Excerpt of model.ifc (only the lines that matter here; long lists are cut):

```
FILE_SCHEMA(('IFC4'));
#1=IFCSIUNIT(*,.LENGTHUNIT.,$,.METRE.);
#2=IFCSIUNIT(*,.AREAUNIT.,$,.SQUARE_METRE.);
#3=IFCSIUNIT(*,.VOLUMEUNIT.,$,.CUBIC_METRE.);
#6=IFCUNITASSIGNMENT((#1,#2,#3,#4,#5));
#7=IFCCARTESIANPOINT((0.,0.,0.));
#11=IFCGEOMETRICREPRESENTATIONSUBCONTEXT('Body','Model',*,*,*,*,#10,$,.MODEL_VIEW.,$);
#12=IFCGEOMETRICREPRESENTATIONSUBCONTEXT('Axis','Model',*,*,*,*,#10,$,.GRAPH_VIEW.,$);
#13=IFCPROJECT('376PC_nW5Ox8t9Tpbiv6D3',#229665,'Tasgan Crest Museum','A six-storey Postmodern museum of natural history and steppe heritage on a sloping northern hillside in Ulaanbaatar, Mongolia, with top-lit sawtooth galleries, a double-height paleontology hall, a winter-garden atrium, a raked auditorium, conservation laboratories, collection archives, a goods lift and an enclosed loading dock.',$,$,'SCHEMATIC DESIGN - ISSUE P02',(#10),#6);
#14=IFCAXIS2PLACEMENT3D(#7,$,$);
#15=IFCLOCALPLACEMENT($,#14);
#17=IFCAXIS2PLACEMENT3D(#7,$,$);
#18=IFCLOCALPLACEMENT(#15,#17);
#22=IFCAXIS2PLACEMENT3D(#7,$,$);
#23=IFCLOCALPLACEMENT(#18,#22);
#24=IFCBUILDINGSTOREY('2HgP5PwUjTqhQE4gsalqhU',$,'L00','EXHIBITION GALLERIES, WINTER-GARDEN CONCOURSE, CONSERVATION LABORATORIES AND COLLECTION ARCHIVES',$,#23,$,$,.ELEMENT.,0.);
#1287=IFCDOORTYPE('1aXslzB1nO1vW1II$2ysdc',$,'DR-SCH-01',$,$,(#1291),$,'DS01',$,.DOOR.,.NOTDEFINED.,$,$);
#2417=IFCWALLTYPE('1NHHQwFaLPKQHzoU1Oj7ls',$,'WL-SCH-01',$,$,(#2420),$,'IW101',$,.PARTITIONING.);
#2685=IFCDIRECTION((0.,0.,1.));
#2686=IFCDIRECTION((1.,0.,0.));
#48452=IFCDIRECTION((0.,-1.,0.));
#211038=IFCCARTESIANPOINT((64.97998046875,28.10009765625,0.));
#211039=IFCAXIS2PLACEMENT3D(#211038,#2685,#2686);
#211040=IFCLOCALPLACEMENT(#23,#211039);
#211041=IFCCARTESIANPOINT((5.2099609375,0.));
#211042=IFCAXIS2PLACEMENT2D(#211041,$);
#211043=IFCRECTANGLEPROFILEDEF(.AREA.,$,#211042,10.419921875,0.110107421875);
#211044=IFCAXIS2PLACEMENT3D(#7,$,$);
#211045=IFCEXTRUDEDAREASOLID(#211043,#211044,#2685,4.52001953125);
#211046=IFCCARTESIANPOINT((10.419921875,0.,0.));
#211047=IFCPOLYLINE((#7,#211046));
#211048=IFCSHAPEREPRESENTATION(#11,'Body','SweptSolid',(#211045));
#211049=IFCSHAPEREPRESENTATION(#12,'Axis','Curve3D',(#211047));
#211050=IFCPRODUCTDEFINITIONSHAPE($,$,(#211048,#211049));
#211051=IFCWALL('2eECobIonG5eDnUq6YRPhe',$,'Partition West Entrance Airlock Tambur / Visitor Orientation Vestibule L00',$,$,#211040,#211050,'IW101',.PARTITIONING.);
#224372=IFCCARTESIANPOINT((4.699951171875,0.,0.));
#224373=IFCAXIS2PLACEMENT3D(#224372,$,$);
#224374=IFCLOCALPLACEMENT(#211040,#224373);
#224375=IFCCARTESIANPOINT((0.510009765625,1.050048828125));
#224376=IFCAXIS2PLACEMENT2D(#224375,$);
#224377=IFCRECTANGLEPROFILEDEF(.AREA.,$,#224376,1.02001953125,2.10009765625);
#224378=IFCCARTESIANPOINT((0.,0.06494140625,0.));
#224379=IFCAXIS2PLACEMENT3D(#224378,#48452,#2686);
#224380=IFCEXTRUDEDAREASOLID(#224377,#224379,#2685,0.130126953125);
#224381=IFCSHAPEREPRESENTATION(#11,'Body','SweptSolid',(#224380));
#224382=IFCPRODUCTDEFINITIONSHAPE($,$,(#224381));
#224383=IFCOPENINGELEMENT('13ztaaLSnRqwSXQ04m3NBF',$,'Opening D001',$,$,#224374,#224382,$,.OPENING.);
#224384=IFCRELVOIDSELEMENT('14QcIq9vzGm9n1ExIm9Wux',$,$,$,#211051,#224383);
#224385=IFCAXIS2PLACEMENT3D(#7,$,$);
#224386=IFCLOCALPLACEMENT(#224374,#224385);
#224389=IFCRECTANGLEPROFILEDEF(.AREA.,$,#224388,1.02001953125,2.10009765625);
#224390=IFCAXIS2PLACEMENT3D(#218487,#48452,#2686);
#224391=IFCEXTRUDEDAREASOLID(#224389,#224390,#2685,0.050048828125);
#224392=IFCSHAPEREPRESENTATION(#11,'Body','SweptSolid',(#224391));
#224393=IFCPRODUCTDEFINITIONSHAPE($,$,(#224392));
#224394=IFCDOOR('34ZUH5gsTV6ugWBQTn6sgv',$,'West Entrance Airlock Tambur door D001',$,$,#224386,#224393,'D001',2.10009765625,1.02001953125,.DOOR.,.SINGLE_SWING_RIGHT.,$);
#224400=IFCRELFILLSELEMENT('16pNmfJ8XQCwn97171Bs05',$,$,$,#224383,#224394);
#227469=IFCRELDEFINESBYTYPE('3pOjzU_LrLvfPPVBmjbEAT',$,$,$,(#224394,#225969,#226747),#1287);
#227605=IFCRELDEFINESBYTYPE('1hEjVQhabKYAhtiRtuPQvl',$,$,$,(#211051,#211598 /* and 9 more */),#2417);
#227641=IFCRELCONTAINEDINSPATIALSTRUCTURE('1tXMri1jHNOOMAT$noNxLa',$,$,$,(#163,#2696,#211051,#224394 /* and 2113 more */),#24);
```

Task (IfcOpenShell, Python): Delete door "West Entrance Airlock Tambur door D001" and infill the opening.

```python
import ifcopenshell
import ifcopenshell.api.feature
import ifcopenshell.api.root
import ifcopenshell.geom
import ifcopenshell.util.shape

model = ifcopenshell.open("model.ifc")
settings = ifcopenshell.geom.settings()


def volume(element):
    """Net volume in cubic metres, openings subtracted."""
    shape = ifcopenshell.geom.create_shape(settings, element)
    return ifcopenshell.util.shape.get_volume(shape.geometry)


door = model.by_guid("34ZUH5gsTV6ugWBQTn6sgv")
opening = door.FillsVoids[0].RelatingOpeningElement
wall = opening.VoidsElements[0].RelatingBuildingElement
before = volume(wall)

ifcopenshell.api.root.remove_product(model, product=door)
ifcopenshell.api.feature.remove_feature(model, feature=opening)

after = volume(wall)

print(f"wall volume {before:.3f} -> {after:.3f} m3")

model.write("model-out.ifc")
```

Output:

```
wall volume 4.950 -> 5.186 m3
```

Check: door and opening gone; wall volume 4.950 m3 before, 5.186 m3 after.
